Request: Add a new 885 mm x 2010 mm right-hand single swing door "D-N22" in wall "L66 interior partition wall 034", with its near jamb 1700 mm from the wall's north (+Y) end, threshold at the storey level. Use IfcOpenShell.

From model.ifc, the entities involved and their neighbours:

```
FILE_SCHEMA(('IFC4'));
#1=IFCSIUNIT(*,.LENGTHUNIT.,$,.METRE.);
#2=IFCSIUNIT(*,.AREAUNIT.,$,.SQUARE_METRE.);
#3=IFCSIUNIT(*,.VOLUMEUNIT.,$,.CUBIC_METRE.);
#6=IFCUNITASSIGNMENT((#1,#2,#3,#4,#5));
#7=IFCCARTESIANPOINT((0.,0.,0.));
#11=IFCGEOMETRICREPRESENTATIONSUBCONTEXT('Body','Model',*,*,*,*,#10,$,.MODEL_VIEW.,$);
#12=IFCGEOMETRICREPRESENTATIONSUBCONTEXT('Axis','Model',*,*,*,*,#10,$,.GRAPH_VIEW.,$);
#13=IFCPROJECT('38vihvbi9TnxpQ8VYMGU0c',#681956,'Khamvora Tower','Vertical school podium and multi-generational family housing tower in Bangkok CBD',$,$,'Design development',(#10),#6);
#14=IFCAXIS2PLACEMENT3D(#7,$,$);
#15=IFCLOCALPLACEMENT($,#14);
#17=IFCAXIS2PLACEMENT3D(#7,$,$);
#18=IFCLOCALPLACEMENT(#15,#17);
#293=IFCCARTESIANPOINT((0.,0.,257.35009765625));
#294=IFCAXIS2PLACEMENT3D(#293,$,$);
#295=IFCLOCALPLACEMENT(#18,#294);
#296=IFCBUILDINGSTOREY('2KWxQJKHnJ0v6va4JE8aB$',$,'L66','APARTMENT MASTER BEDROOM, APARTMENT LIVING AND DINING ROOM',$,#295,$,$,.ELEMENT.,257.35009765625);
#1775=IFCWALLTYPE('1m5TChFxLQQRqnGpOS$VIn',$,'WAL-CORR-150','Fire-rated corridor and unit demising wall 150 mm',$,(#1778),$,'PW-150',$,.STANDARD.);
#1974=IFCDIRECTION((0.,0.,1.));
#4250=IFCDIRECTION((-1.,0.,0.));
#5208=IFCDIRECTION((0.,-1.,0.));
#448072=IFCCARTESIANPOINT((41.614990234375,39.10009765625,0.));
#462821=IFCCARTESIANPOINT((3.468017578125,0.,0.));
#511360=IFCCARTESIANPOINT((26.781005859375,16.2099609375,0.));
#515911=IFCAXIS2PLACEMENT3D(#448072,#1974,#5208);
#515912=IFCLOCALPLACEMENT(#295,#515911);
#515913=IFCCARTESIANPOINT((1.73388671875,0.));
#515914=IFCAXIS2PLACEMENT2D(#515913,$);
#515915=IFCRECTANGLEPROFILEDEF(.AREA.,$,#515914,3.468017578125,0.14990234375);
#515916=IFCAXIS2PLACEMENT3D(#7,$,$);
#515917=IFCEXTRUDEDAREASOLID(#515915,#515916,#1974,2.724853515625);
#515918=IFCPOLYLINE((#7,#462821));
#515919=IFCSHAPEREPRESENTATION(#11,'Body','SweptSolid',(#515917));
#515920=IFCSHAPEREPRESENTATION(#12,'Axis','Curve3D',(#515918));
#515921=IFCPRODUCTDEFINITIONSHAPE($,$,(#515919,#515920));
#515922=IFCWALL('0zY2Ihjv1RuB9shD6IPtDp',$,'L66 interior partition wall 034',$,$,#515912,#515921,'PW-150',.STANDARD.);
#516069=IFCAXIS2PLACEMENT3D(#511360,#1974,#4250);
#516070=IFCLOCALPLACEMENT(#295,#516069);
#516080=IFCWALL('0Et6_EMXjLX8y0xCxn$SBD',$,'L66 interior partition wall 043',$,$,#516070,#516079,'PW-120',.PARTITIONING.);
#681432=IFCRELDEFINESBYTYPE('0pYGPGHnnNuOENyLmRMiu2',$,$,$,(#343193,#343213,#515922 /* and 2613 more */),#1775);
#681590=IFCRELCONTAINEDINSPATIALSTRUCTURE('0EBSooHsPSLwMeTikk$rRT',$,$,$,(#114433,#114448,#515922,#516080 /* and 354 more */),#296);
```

```python
import numpy as np
import ifcopenshell
import ifcopenshell.api.feature
import ifcopenshell.api.geometry
import ifcopenshell.api.root
import ifcopenshell.api.spatial
import ifcopenshell.geom
import ifcopenshell.util.element
import ifcopenshell.util.placement
import ifcopenshell.util.representation
import ifcopenshell.util.shape
import ifcopenshell.util.unit

model = ifcopenshell.open("model.ifc")
unit_scale = ifcopenshell.util.unit.calculate_unit_scale(model)
settings = ifcopenshell.geom.settings()


def volume(element):
    """Net volume in cubic metres, openings subtracted."""
    shape = ifcopenshell.geom.create_shape(settings, element)
    return ifcopenshell.util.shape.get_volume(shape.geometry)


wall = model.by_guid("0zY2Ihjv1RuB9shD6IPtDp")
storey = ifcopenshell.util.element.get_container(wall, ifc_class="IfcBuildingStorey")
context = ifcopenshell.util.representation.get_context(model, "Model", "Body", "MODEL_VIEW")
before = volume(wall)

width, height, from_end, sill = 0.885, 2.01, 1.7, 0.0  # metres

# The wall runs along its own X axis, and the end named is its -X end.
wall_shape = ifcopenshell.geom.create_shape(settings, wall)
x, y, z = ifcopenshell.util.shape.get_vertices(wall_shape.geometry).T
start = x.min() + from_end
face, thickness = float(y.min()), float(y.max() - y.min())
wall_matrix = ifcopenshell.util.placement.get_local_placement(wall.ObjectPlacement)
level = ifcopenshell.util.placement.get_local_placement(storey.ObjectPlacement)[2, 3]


def in_wall(x, y):
    """Placement at x, y metres in the wall's axes, at sill height."""
    matrix = wall_matrix.copy()
    matrix[:, 3] = wall_matrix @ np.array([x / unit_scale, y / unit_scale, 0.0, 1.0])
    matrix[2, 3] = level + sill / unit_scale
    return matrix


# Opening: a box that overshoots both wall faces by 50 mm.
opening = ifcopenshell.api.root.create_entity(model, ifc_class="IfcOpeningElement", predefined_type="OPENING")
box = ifcopenshell.api.geometry.add_wall_representation(
    model, context=context, length=width, height=height, thickness=thickness + 0.1
)
ifcopenshell.api.geometry.assign_representation(model, product=opening, representation=box)
ifcopenshell.api.geometry.edit_object_placement(model, product=opening, matrix=in_wall(start, face - 0.05), is_si=False)
ifcopenshell.api.feature.add_feature(model, feature=opening, element=wall)

door = ifcopenshell.api.root.create_entity(model, ifc_class="IfcDoor", name="D-N22", predefined_type="DOOR")
door.OverallWidth, door.OverallHeight = width / unit_scale, height / unit_scale
door.OperationType = "SINGLE_SWING_RIGHT"
body = ifcopenshell.api.geometry.add_door_representation(
    model,
    context=context,
    overall_width=door.OverallWidth,
    overall_height=door.OverallHeight,
    operation_type="SINGLE_SWING_RIGHT",
    lining_properties={"LiningDepth": thickness / unit_scale, "ThresholdDepth": thickness / unit_scale},
)
ifcopenshell.api.geometry.assign_representation(model, product=door, representation=body)
ifcopenshell.api.spatial.assign_container(model, products=[door], relating_structure=storey)
ifcopenshell.api.feature.add_filling(model, opening=opening, element=door)

# The lining spans the wall, so the door starts at the wall face.
ifcopenshell.api.geometry.edit_object_placement(model, product=door, matrix=in_wall(start, face), is_si=False)

after = volume(wall)

print(f"wall volume {before:.3f} -> {after:.3f} m3")

model.write("model_v2.ifc")
```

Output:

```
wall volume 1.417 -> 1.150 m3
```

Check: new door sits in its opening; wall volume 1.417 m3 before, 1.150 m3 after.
